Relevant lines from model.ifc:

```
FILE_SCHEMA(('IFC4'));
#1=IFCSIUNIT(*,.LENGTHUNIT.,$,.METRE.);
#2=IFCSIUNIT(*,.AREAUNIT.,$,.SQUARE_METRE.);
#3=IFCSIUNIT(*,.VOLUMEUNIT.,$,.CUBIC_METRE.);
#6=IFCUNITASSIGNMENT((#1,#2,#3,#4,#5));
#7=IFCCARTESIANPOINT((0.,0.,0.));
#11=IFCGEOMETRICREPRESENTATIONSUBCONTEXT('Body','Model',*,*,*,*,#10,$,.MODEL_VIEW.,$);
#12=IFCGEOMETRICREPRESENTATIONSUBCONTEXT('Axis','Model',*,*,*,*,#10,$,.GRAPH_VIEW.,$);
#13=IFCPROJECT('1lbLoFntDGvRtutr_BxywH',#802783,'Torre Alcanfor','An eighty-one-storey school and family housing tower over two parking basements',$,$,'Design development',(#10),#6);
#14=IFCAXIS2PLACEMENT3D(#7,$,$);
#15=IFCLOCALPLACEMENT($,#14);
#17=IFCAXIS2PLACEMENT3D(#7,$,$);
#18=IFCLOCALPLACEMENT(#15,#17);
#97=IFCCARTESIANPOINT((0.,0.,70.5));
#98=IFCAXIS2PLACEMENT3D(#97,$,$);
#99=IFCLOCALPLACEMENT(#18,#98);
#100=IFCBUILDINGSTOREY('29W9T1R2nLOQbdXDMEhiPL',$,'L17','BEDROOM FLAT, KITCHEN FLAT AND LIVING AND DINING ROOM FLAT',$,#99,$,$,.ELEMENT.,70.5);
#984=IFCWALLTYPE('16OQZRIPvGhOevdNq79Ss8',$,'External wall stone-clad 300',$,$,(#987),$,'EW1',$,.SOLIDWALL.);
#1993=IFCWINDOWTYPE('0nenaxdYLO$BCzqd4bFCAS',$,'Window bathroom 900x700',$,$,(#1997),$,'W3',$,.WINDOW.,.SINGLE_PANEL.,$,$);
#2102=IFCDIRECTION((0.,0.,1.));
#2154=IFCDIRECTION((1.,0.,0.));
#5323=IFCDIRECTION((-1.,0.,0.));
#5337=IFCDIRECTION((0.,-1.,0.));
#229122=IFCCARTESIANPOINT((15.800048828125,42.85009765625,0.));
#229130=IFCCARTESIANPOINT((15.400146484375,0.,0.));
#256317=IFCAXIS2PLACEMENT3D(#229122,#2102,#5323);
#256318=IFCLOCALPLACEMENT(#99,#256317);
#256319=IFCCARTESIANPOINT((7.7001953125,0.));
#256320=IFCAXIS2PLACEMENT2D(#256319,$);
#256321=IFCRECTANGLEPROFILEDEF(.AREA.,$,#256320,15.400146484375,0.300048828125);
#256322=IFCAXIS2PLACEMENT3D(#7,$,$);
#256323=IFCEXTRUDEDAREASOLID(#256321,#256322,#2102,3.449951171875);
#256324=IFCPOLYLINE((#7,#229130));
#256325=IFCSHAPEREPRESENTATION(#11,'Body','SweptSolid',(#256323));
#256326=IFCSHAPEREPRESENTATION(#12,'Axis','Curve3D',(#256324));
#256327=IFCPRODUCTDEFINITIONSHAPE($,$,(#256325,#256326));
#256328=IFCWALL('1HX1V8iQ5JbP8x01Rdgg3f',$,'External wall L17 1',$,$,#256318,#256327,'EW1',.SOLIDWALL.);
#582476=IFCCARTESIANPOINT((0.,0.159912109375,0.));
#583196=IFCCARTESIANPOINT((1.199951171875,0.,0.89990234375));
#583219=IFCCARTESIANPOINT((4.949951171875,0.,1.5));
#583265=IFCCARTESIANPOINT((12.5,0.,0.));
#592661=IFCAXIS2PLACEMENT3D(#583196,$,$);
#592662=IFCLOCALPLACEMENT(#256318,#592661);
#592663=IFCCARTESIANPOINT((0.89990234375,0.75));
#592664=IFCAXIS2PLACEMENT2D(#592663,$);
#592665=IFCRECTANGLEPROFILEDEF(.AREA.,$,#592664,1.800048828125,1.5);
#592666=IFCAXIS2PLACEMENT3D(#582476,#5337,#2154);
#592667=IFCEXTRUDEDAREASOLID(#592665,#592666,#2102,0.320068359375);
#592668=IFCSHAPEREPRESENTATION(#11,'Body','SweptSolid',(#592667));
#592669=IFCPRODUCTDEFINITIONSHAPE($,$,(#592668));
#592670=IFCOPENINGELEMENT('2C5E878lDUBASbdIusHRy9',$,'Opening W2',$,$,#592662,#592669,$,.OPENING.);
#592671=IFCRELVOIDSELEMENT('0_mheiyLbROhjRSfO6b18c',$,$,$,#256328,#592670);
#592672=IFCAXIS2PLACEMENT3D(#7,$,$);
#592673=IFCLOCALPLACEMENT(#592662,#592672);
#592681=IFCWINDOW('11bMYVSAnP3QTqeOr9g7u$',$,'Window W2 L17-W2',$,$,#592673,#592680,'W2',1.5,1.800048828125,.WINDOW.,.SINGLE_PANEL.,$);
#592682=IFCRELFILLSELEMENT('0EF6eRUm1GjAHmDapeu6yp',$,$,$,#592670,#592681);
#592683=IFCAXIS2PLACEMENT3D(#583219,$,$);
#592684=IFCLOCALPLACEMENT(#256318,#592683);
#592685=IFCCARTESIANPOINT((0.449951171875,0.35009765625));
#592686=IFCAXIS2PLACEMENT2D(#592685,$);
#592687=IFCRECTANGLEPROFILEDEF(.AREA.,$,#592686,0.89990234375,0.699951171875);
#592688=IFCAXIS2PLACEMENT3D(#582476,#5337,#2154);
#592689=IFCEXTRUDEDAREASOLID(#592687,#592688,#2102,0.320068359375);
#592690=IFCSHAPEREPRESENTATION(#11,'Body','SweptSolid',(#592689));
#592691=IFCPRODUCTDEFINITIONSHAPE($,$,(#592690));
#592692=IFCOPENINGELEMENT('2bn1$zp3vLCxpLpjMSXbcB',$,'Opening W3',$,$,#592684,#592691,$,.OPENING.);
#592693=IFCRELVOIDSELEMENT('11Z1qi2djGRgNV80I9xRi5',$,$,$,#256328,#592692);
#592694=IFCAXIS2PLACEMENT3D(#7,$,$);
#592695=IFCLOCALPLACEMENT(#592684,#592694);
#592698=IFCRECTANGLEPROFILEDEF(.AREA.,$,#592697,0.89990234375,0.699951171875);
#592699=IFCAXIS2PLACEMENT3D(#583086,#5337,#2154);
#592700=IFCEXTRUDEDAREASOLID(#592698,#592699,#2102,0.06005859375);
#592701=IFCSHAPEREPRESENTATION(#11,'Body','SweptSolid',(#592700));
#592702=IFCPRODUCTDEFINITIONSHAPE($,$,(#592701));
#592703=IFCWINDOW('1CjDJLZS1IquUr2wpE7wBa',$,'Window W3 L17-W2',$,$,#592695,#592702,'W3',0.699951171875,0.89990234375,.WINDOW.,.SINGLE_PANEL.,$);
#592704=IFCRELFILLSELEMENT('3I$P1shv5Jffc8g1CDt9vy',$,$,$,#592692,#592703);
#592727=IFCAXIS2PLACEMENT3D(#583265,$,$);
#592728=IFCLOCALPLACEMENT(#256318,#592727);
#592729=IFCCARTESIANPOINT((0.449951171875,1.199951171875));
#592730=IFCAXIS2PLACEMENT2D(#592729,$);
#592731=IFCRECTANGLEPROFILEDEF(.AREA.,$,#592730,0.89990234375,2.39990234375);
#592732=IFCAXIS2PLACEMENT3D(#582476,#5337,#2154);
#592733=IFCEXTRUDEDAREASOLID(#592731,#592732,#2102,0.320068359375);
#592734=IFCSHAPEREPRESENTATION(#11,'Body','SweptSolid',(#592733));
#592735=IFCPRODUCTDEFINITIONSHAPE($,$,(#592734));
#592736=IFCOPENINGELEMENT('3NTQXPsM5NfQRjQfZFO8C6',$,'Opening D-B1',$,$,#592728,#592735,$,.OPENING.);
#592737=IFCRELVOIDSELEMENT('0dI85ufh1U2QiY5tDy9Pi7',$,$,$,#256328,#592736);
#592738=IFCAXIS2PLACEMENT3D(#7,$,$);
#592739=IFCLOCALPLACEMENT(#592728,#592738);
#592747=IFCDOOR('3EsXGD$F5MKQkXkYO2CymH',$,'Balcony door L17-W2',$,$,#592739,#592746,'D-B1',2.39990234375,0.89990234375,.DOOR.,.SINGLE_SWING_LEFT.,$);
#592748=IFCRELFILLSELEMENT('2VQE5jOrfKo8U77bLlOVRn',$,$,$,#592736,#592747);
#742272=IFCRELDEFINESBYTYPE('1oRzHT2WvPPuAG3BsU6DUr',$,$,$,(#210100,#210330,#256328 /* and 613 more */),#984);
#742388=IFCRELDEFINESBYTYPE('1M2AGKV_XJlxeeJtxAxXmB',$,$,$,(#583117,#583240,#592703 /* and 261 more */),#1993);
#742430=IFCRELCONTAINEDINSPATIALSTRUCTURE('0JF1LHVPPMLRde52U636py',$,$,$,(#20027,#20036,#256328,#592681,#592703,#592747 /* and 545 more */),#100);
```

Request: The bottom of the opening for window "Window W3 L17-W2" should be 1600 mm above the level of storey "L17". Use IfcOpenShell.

```python
import numpy as np
import ifcopenshell
import ifcopenshell.api.geometry
import ifcopenshell.geom
import ifcopenshell.util.element
import ifcopenshell.util.placement
import ifcopenshell.util.shape
import ifcopenshell.util.unit

model = ifcopenshell.open("model.ifc")
unit_scale = ifcopenshell.util.unit.calculate_unit_scale(model)

window = model.by_id(592703)
opening = window.FillsVoids[0].RelatingOpeningElement
storey = ifcopenshell.util.element.get_container(window, ifc_class="IfcBuildingStorey")
level = ifcopenshell.util.placement.get_local_placement(storey.ObjectPlacement)[2, 3]

# The opening's origin need not be at the sill, so measure its lowest point.
shape = ifcopenshell.geom.create_shape(ifcopenshell.geom.settings(), opening)
bottom = ifcopenshell.util.shape.get_shape_bottom_elevation(shape, shape.geometry) / unit_scale
dz = level + 1.6 / unit_scale - bottom

shift = np.array([0.0, 0.0, dz])
# The window is placed relative to its opening, so it follows when the opening moves.
matrix = ifcopenshell.util.placement.get_local_placement(opening.ObjectPlacement)
matrix[:3, 3] += shift
ifcopenshell.api.geometry.edit_object_placement(
    model, product=opening, matrix=matrix, is_si=False, should_transform_children=True
)

print(f"moved by {dz * unit_scale:+.3f} m")

model.write("model_updated.ifc")
```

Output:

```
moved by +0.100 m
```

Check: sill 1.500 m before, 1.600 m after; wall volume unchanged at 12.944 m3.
